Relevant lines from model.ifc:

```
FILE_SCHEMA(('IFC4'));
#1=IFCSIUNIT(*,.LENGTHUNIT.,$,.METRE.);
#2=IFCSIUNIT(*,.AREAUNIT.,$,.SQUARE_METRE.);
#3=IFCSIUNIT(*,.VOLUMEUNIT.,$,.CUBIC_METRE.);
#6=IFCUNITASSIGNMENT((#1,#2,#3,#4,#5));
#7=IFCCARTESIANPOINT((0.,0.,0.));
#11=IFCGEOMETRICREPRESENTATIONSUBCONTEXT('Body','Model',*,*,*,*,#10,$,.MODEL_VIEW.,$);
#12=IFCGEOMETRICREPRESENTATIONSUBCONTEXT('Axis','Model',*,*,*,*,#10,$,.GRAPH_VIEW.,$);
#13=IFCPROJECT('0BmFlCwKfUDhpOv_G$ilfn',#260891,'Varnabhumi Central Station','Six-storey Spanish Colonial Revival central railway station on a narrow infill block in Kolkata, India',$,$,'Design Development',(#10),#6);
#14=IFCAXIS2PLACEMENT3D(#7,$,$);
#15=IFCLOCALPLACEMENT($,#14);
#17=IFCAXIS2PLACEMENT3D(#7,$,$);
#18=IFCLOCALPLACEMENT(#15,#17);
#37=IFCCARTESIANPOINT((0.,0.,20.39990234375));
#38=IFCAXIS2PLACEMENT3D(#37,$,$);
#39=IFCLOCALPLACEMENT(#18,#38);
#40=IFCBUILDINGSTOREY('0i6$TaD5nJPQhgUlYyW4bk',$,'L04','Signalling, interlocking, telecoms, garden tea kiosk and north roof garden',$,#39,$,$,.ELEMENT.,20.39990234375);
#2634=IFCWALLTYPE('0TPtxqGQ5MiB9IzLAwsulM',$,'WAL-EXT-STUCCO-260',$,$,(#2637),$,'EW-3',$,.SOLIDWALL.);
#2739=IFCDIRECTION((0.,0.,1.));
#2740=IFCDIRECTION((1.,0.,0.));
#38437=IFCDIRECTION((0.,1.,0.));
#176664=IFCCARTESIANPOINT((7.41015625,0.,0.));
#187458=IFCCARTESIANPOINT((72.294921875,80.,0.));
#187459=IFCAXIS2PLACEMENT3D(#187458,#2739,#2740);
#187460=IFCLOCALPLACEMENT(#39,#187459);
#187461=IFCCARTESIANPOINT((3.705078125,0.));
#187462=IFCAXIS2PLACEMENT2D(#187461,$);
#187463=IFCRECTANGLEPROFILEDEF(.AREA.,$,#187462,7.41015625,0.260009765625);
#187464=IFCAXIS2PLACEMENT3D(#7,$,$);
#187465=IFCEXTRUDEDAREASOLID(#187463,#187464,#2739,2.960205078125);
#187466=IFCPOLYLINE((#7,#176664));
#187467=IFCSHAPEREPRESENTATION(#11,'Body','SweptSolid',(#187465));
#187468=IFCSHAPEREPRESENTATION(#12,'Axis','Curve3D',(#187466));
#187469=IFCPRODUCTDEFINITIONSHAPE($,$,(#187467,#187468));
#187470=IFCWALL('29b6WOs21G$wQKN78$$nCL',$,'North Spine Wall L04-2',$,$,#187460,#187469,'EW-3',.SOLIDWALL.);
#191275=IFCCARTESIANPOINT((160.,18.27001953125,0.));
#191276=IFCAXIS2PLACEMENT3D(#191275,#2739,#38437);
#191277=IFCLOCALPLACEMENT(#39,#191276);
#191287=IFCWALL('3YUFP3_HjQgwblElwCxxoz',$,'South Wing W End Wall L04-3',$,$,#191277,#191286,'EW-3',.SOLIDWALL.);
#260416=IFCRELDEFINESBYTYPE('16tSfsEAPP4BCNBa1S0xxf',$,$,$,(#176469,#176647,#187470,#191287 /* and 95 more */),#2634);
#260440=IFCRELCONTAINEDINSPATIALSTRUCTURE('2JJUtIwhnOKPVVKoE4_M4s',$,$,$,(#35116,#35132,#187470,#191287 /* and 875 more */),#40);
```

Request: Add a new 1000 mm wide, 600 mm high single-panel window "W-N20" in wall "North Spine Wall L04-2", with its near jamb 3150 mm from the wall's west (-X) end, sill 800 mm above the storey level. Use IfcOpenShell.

```python
import numpy as np
import ifcopenshell
import ifcopenshell.api.feature
import ifcopenshell.api.geometry
import ifcopenshell.api.root
import ifcopenshell.api.spatial
import ifcopenshell.geom
import ifcopenshell.util.element
import ifcopenshell.util.placement
import ifcopenshell.util.representation
import ifcopenshell.util.shape
import ifcopenshell.util.unit

model = ifcopenshell.open("model.ifc")
unit_scale = ifcopenshell.util.unit.calculate_unit_scale(model)
settings = ifcopenshell.geom.settings()


def volume(element):
    """Net volume in cubic metres, openings subtracted."""
    shape = ifcopenshell.geom.create_shape(settings, element)
    return ifcopenshell.util.shape.get_volume(shape.geometry)


wall = model.by_guid("29b6WOs21G$wQKN78$$nCL")
storey = ifcopenshell.util.element.get_container(wall, ifc_class="IfcBuildingStorey")
context = ifcopenshell.util.representation.get_context(model, "Model", "Body", "MODEL_VIEW")
before = volume(wall)

width, height, from_end, sill = 1, 0.6, 3.15, 0.8  # metres

# The wall runs along its own X axis, and the end named is its -X end.
wall_shape = ifcopenshell.geom.create_shape(settings, wall)
x, y, z = ifcopenshell.util.shape.get_vertices(wall_shape.geometry).T
start = x.min() + from_end
face, thickness = float(y.min()), float(y.max() - y.min())
wall_matrix = ifcopenshell.util.placement.get_local_placement(wall.ObjectPlacement)
level = ifcopenshell.util.placement.get_local_placement(storey.ObjectPlacement)[2, 3]


def in_wall(x, y):
    """Placement at x, y metres in the wall's axes, at sill height."""
    matrix = wall_matrix.copy()
    matrix[:, 3] = wall_matrix @ np.array([x / unit_scale, y / unit_scale, 0.0, 1.0])
    matrix[2, 3] = level + sill / unit_scale
    return matrix


# Opening: a box that overshoots both wall faces by 50 mm.
opening = ifcopenshell.api.root.create_entity(model, ifc_class="IfcOpeningElement", predefined_type="OPENING")
box = ifcopenshell.api.geometry.add_wall_representation(
    model, context=context, length=width, height=height, thickness=thickness + 0.1
)
ifcopenshell.api.geometry.assign_representation(model, product=opening, representation=box)
ifcopenshell.api.geometry.edit_object_placement(model, product=opening, matrix=in_wall(start, face - 0.05), is_si=False)
ifcopenshell.api.feature.add_feature(model, feature=opening, element=wall)

window = ifcopenshell.api.root.create_entity(model, ifc_class="IfcWindow", name="W-N20", predefined_type="WINDOW")
window.OverallWidth, window.OverallHeight = width / unit_scale, height / unit_scale
window.PartitioningType = "SINGLE_PANEL"
body = ifcopenshell.api.geometry.add_window_representation(
    model,
    context=context,
    overall_width=window.OverallWidth,
    overall_height=window.OverallHeight,
    partition_type="SINGLE_PANEL",
)
ifcopenshell.api.geometry.assign_representation(model, product=window, representation=body)
ifcopenshell.api.spatial.assign_container(model, products=[window], relating_structure=storey)
ifcopenshell.api.feature.add_filling(model, opening=opening, element=window)

# Centre the window in the wall's thickness.
ifcopenshell.api.geometry.edit_object_placement(model, product=window, matrix=in_wall(start, face), is_si=False)
window_shape = ifcopenshell.geom.create_shape(settings, window)
depth = ifcopenshell.util.shape.get_vertices(window_shape.geometry)[:, 1]
offset = face + thickness / 2 - (depth.min() + depth.max()) / 2
ifcopenshell.api.geometry.edit_object_placement(model, product=window, matrix=in_wall(start, offset), is_si=False)

after = volume(wall)

print(f"wall volume {before:.3f} -> {after:.3f} m3")

model.write("model_edited.ifc")
```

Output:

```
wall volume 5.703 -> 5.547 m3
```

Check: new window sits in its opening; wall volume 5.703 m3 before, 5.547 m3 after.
